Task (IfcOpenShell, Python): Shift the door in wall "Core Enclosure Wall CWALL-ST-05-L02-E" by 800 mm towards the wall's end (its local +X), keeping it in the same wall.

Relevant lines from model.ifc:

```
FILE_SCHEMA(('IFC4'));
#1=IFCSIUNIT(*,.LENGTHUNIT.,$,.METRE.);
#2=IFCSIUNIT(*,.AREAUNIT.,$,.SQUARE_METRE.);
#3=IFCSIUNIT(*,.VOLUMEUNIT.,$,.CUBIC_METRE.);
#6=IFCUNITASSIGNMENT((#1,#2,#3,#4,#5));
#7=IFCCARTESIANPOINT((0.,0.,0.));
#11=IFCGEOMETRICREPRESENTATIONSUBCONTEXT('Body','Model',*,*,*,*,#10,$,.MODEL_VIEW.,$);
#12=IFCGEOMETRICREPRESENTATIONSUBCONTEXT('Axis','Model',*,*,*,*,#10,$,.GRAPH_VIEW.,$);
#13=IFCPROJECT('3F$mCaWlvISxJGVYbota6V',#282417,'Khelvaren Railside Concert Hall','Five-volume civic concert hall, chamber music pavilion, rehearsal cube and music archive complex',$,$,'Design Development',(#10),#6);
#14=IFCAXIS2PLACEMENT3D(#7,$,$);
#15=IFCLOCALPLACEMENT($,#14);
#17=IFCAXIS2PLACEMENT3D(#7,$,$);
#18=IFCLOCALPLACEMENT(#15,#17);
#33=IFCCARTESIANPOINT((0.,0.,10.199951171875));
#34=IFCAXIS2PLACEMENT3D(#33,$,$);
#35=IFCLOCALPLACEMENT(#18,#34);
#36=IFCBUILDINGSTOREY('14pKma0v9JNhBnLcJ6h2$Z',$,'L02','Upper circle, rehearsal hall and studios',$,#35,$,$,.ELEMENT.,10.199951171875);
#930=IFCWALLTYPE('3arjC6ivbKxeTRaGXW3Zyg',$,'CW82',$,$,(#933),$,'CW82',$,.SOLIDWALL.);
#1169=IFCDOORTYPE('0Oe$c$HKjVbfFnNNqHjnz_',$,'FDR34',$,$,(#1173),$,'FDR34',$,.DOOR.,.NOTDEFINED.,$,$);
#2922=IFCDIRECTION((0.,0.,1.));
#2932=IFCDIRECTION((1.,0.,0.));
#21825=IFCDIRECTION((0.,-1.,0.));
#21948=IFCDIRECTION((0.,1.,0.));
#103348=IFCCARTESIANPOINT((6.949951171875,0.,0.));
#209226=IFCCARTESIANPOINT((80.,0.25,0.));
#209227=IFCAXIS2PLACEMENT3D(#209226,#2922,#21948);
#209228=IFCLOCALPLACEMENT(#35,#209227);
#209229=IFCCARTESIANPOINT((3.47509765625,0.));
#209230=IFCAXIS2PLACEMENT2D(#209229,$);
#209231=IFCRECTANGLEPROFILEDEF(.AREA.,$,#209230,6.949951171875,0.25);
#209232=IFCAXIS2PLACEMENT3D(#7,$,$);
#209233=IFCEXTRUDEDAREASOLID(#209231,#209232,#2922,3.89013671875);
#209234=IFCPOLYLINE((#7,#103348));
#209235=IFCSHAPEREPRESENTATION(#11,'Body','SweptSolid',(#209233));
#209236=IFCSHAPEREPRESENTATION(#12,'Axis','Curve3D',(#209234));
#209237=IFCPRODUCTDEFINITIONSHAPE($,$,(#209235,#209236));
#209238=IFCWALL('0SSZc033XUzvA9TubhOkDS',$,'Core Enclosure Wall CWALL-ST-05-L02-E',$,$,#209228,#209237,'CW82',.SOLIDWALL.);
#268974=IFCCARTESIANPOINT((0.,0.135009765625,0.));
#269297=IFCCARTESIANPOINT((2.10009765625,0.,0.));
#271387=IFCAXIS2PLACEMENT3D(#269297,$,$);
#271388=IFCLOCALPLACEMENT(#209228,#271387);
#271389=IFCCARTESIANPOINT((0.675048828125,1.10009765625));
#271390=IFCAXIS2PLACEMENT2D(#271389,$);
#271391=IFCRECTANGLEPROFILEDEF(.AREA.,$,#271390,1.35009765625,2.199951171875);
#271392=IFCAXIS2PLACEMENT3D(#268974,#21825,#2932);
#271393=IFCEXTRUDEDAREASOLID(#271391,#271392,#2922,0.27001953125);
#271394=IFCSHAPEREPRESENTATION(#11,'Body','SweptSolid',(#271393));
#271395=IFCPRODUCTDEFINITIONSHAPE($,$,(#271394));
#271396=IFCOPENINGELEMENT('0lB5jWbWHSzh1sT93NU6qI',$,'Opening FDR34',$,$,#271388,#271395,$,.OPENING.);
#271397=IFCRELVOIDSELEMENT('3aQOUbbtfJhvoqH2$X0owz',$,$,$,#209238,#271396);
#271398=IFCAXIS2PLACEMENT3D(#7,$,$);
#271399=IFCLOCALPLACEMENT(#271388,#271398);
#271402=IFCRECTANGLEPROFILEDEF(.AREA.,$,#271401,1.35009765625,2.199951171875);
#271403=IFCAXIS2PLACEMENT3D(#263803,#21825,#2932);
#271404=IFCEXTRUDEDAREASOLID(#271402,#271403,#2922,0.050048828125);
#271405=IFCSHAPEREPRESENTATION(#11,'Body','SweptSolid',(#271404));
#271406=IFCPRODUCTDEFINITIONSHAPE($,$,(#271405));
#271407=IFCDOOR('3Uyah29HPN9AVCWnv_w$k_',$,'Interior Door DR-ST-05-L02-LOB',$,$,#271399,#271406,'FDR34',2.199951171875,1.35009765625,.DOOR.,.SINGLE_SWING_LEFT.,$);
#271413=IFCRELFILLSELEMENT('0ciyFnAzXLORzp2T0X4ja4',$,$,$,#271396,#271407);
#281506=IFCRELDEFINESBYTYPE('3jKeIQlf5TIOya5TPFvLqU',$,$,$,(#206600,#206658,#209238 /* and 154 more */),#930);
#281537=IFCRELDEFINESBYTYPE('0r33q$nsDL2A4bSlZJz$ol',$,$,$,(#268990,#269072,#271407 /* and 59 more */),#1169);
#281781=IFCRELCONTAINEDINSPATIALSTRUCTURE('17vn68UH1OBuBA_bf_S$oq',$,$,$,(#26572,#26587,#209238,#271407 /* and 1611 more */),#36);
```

```python
import ifcopenshell
import ifcopenshell.api.geometry
import ifcopenshell.util.placement

model = ifcopenshell.open("model.ifc")

door = model.by_guid("3Uyah29HPN9AVCWnv_w$k_")
opening = door.FillsVoids[0].RelatingOpeningElement
wall = opening.VoidsElements[0].RelatingBuildingElement

wall_matrix = ifcopenshell.util.placement.get_local_placement(wall.ObjectPlacement)
shift = wall_matrix[:3, 0] * 0.8
before = ifcopenshell.util.placement.get_local_placement(door.ObjectPlacement)[:3, 3].copy()

# The door is placed relative to its opening, so it follows when the opening moves.
matrix = ifcopenshell.util.placement.get_local_placement(opening.ObjectPlacement)
matrix[:3, 3] += shift
ifcopenshell.api.geometry.edit_object_placement(
    model, product=opening, matrix=matrix, is_si=False, should_transform_children=True
)

after = ifcopenshell.util.placement.get_local_placement(door.ObjectPlacement)[:3, 3]
print("door moved by", (after - before).round(3) + 0.0)

model.write("model_v2.ifc")
```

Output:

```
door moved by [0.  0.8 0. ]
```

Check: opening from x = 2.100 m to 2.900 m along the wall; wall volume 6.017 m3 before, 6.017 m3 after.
